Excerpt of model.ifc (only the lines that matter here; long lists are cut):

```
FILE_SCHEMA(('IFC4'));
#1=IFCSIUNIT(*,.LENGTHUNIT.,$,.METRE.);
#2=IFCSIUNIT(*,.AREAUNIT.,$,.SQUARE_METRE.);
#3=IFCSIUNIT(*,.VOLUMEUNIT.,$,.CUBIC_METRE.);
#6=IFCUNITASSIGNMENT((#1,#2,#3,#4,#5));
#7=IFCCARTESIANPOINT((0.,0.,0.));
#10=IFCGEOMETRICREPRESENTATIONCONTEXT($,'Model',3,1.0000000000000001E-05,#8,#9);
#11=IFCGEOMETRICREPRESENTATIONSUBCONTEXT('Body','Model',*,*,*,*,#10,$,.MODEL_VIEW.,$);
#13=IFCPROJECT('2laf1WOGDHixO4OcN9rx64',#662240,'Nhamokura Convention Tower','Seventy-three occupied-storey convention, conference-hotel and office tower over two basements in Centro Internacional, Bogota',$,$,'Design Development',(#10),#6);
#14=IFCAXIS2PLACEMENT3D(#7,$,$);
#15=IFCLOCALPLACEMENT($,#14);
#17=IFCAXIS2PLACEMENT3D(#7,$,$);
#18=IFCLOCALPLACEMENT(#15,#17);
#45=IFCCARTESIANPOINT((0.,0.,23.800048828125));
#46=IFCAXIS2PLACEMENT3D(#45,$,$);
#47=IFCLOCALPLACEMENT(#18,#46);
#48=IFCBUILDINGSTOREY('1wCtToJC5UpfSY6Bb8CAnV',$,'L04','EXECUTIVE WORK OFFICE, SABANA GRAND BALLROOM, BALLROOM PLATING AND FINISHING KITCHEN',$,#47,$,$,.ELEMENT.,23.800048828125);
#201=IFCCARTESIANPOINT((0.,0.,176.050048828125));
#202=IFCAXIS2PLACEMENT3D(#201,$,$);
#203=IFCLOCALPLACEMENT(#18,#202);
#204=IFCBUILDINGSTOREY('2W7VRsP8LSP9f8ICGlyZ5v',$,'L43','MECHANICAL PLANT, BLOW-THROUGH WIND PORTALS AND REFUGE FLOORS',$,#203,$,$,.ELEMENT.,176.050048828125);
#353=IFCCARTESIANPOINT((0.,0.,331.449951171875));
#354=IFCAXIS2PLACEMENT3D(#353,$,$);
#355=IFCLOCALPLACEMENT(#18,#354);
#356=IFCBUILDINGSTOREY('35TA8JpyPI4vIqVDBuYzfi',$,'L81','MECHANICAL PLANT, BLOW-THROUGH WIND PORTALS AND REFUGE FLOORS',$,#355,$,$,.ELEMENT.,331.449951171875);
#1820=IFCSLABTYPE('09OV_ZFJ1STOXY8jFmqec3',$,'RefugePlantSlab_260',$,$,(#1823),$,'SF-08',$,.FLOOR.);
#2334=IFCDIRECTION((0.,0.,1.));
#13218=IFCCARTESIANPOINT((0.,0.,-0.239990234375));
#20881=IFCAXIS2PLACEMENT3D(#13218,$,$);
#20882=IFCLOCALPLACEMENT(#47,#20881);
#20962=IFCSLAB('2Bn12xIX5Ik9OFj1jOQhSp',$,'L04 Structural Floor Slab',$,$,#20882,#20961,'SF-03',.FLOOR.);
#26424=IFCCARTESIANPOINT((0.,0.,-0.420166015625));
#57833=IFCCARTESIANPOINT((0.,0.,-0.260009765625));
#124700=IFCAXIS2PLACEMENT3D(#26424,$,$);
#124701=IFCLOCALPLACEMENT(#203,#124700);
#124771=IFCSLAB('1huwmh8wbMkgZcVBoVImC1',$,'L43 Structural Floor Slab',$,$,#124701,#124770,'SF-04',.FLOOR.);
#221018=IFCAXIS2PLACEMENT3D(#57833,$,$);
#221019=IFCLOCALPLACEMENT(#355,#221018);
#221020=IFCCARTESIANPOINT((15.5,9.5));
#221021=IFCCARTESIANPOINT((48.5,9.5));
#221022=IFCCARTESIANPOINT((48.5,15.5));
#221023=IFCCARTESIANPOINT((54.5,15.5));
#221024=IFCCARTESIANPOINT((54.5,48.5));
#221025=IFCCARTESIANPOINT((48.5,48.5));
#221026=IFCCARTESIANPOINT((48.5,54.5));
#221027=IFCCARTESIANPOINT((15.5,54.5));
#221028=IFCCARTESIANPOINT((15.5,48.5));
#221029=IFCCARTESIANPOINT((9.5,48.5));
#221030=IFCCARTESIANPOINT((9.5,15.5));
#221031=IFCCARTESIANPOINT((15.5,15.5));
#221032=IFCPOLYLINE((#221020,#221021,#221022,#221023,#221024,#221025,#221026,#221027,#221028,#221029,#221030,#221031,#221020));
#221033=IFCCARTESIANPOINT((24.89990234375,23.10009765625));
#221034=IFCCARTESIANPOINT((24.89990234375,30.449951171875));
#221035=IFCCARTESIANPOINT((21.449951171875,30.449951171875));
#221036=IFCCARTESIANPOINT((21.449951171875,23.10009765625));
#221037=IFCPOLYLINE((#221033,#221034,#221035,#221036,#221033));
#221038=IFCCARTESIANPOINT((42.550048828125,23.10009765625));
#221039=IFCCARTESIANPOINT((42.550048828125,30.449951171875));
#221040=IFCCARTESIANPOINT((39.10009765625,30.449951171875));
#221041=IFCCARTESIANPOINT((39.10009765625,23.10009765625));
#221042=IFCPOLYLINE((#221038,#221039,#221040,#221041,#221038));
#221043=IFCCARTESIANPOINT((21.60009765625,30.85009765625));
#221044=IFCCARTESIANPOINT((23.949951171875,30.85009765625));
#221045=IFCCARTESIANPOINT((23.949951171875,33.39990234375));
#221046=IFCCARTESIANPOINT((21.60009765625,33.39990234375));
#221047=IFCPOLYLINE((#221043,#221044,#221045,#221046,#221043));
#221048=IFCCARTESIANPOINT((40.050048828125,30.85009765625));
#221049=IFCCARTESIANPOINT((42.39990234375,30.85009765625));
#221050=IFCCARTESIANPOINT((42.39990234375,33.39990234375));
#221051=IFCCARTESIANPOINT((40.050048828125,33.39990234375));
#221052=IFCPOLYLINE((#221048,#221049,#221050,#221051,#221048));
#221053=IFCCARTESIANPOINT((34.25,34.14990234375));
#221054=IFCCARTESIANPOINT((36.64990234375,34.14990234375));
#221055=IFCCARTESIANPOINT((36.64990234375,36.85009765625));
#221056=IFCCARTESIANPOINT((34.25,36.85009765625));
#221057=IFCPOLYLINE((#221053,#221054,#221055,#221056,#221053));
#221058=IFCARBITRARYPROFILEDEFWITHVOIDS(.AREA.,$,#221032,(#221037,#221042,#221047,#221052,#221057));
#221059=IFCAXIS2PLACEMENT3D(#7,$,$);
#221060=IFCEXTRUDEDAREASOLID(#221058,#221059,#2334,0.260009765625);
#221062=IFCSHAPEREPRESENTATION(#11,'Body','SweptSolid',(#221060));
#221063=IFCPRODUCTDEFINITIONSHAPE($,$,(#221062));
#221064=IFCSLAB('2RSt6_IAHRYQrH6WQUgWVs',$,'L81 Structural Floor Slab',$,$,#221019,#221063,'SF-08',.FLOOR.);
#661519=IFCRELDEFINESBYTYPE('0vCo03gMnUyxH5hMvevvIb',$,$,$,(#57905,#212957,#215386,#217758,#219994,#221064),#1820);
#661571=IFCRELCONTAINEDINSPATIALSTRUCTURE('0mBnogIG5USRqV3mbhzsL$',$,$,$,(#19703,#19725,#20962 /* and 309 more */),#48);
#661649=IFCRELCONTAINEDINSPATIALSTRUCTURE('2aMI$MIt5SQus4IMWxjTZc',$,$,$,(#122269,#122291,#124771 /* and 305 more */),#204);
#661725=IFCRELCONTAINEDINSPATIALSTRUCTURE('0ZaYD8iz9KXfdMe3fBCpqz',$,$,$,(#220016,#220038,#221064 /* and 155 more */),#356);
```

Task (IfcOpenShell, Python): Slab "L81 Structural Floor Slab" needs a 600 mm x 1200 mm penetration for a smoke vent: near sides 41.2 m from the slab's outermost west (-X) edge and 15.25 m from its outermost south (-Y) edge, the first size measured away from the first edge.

```python
import numpy as np
import ifcopenshell
import ifcopenshell.api.feature
import ifcopenshell.api.geometry
import ifcopenshell.api.root
import ifcopenshell.geom
import ifcopenshell.util.placement
import ifcopenshell.util.representation
import ifcopenshell.util.shape
import ifcopenshell.util.unit

model = ifcopenshell.open("model.ifc")
unit_scale = ifcopenshell.util.unit.calculate_unit_scale(model)
settings = ifcopenshell.geom.settings()


def volume(element):
    """Net volume in cubic metres, openings subtracted."""
    shape = ifcopenshell.geom.create_shape(settings, element)
    return ifcopenshell.util.shape.get_volume(shape.geometry)


slab = model.by_id(221064)
before = volume(slab)

# Extent in the slab's own axes, in metres. The edges named are its -X and -Y sides.
slab_shape = ifcopenshell.geom.create_shape(settings, slab)
vertices = ifcopenshell.util.shape.get_vertices(slab_shape.geometry)
x_min, y_min, bottom = vertices.min(axis=0)
top = vertices[:, 2].max()

opening = ifcopenshell.api.root.create_entity(model, ifc_class="IfcOpeningElement", name="Smoke vent opening", predefined_type="OPENING")
context = ifcopenshell.util.representation.get_context(model, "Model", "Body", "MODEL_VIEW")
width, depth = 0.6, 1.2
outline = [(0.0, 0.0), (width, 0.0), (width, depth), (0.0, depth), (0.0, 0.0)]
# Overshoot both faces by 50 mm so the cut is clean.
shape = ifcopenshell.api.geometry.add_slab_representation(
    model, context=context, depth=top - bottom + 0.1, polyline=outline
)
ifcopenshell.api.geometry.assign_representation(model, product=opening, representation=shape)

matrix = ifcopenshell.util.placement.get_local_placement(slab.ObjectPlacement)
matrix[:, 3] = matrix @ np.append(np.array([x_min + 41.2, y_min + 15.25, bottom - 0.05]) / unit_scale, 1.0)
ifcopenshell.api.geometry.edit_object_placement(model, product=opening, matrix=matrix, is_si=False)
ifcopenshell.api.feature.add_feature(model, feature=opening, element=slab)

after = volume(slab)

print(f"slab volume {before:.3f} -> {after:.3f} m3")

model.write("model_edited.ifc")
```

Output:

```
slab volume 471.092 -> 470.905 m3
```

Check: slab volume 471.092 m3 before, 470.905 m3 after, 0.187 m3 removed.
